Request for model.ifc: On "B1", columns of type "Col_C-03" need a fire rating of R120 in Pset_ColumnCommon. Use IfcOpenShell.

First a look at what the model holds.

```python
import ifcopenshell
import ifcopenshell.util.element

model = ifcopenshell.open("model.ifc")
print(model.schema)
storey = next(s for s in model.by_type("IfcBuildingStorey") if s.Name == "B1")
columns = [e for e in ifcopenshell.util.element.get_decomposition(storey) if e.is_a("IfcColumn")]
seen = {}
for e in columns:
    element_type = ifcopenshell.util.element.get_type(e)
    key = (element_type.Name if element_type != e and element_type else None, ifcopenshell.util.element.get_pset(e, "Pset_ColumnCommon", "FireRating"))
    seen[key] = seen.get(key, 0) + 1
for (name, value), count in sorted(seen.items(), key=str):
    print(count, "x", name, "|", value)
```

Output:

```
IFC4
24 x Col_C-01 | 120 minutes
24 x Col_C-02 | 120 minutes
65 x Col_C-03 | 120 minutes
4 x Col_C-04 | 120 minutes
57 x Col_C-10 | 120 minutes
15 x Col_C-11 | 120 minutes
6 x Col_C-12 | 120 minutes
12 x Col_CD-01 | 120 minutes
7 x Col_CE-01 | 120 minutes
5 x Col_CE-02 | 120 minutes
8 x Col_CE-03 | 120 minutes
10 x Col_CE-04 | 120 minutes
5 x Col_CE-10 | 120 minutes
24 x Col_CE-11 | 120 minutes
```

```python
import ifcopenshell
import ifcopenshell.api.pset
import ifcopenshell.util.element

model = ifcopenshell.open("model.ifc")

storey = next(s for s in model.by_type("IfcBuildingStorey") if s.Name == "B1")
columns = [e for e in ifcopenshell.util.element.get_decomposition(storey) if e.is_a("IfcColumn")]

count = 0
for e in columns:
    element_type = ifcopenshell.util.element.get_type(e)
    if element_type in (None, e) or element_type.Name != "Col_C-03":
        continue
    # add_pset returns the element's existing set when there is one.
    pset = ifcopenshell.api.pset.add_pset(model, product=e, name="Pset_ColumnCommon")
    ifcopenshell.api.pset.edit_pset(model, pset=pset, properties={"FireRating": "R120"})
    count += 1

print(count, "columns updated")

model.write("model_v2.ifc")
```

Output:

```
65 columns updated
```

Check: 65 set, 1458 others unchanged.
